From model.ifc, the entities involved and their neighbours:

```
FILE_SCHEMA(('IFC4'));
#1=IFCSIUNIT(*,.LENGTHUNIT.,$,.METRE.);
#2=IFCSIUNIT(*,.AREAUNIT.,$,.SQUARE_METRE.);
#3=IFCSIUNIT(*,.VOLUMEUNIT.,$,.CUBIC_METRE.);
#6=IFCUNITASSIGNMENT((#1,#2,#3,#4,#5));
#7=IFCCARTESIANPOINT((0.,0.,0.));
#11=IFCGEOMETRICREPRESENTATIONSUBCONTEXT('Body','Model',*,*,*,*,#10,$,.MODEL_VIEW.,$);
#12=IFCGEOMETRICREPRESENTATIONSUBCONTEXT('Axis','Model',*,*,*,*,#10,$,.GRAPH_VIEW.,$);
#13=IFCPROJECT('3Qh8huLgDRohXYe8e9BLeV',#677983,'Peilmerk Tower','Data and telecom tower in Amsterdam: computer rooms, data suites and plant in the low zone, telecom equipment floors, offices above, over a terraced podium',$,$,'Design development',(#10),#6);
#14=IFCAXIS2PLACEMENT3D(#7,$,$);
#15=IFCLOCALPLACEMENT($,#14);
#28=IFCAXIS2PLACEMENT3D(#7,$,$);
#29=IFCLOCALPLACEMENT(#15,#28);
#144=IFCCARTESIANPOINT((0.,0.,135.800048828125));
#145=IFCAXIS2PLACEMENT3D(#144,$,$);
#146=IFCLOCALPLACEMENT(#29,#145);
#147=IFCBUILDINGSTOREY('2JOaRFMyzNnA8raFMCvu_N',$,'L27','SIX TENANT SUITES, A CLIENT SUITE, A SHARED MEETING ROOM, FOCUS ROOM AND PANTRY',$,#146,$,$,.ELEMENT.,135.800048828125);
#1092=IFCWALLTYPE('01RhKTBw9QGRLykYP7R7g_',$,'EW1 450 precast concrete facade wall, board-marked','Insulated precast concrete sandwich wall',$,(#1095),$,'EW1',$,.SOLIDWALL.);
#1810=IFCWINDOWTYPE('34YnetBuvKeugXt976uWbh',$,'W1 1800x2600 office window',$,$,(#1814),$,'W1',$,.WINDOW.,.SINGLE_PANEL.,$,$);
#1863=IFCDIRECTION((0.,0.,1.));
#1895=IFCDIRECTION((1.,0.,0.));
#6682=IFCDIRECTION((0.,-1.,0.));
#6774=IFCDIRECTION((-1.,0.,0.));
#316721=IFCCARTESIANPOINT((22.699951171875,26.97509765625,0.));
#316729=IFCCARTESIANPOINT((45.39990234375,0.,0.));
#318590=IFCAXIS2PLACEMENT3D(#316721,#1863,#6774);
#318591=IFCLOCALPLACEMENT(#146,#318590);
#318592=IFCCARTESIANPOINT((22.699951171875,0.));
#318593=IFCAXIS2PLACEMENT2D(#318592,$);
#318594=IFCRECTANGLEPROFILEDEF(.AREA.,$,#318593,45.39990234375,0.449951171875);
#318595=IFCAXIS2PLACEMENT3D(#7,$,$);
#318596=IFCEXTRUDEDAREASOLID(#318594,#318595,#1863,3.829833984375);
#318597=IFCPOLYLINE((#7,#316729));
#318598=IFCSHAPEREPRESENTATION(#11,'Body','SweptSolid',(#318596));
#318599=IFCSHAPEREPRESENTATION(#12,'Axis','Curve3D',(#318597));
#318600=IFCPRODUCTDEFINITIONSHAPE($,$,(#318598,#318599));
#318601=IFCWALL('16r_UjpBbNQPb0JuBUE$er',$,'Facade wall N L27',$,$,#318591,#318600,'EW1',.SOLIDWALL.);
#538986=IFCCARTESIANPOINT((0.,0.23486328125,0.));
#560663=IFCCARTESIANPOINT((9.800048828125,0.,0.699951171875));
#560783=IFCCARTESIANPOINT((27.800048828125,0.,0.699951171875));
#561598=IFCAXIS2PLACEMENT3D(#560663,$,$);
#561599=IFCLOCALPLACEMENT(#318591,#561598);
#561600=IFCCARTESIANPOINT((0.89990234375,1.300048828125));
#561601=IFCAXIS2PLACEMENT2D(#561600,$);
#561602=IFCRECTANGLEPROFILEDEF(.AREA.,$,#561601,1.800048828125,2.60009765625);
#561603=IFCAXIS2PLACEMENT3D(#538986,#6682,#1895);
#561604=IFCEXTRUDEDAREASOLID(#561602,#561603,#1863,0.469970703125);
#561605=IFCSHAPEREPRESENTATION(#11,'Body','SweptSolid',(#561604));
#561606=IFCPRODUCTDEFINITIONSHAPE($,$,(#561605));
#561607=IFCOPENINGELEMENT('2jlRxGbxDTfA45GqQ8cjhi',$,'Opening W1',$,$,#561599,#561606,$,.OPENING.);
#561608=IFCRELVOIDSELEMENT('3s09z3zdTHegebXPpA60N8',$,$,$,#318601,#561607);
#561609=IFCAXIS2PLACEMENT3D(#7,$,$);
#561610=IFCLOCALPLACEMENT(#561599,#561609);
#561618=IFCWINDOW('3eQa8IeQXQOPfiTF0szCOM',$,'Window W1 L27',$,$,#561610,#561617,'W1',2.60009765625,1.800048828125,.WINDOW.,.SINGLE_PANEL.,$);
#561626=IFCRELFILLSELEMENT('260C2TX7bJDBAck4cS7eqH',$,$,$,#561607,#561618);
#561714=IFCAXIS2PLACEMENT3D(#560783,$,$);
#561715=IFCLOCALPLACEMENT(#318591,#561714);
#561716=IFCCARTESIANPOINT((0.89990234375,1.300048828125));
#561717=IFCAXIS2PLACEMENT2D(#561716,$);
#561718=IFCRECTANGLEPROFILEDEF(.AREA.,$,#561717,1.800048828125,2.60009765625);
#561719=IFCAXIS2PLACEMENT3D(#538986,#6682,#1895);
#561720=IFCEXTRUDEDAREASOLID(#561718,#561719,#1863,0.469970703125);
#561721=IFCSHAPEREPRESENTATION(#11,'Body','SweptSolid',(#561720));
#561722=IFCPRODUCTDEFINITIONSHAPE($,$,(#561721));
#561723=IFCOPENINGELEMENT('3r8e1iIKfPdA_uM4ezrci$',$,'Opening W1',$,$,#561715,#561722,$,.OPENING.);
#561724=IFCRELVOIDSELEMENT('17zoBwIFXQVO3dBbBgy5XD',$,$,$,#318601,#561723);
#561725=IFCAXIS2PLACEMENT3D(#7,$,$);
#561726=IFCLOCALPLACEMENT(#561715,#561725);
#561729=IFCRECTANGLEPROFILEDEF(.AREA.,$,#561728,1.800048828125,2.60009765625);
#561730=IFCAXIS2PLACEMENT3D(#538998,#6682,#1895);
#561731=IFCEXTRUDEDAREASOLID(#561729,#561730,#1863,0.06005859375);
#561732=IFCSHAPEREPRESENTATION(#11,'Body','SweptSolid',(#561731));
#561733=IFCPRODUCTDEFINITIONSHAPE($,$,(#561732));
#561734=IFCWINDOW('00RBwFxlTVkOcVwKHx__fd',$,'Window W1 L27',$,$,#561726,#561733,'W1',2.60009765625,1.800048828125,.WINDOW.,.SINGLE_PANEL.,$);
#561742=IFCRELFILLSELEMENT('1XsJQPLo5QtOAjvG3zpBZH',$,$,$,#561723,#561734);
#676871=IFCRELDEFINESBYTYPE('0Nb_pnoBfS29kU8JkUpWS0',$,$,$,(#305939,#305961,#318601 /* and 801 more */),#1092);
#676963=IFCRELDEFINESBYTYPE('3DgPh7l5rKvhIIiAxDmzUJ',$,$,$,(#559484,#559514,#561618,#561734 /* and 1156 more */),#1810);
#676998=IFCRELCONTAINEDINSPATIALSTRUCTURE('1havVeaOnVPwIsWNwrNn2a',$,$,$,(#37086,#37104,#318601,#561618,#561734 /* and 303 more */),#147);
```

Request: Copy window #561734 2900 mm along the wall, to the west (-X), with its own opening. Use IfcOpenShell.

```python
import ifcopenshell
import ifcopenshell.api.feature
import ifcopenshell.api.geometry
import ifcopenshell.api.root
import ifcopenshell.geom
import ifcopenshell.util.element
import ifcopenshell.util.placement
import ifcopenshell.util.shape
import ifcopenshell.util.unit

model = ifcopenshell.open("model.ifc")
unit_scale = ifcopenshell.util.unit.calculate_unit_scale(model)
settings = ifcopenshell.geom.settings()


def volume(element):
    """Net volume in cubic metres, openings subtracted."""
    shape = ifcopenshell.geom.create_shape(settings, element)
    return ifcopenshell.util.shape.get_volume(shape.geometry)


window = model.by_guid("00RBwFxlTVkOcVwKHx__fd")
opening = window.FillsVoids[0].RelatingOpeningElement
wall = opening.VoidsElements[0].RelatingBuildingElement
before = volume(wall)
shift = ifcopenshell.util.placement.get_local_placement(wall.ObjectPlacement)[:3, 0] * 2.9 / unit_scale

# copy_class copies the void relationship, type, container and properties, but no geometry.
new_opening = ifcopenshell.api.root.copy_class(model, product=opening)
new_opening.Representation = ifcopenshell.util.element.copy_deep(
    model, opening.Representation, exclude=["IfcGeometricRepresentationContext", "IfcRepresentationMap"]
)
new_window = ifcopenshell.api.root.copy_class(model, product=window)
new_window.Representation = ifcopenshell.util.element.copy_deep(
    model, window.Representation, exclude=["IfcGeometricRepresentationContext", "IfcRepresentationMap"]
)
new_window.Tag = None
ifcopenshell.api.feature.add_filling(model, opening=new_opening, element=new_window)

for old, new in ((opening, new_opening), (window, new_window)):
    matrix = ifcopenshell.util.placement.get_local_placement(old.ObjectPlacement)
    matrix[:3, 3] += shift
    ifcopenshell.api.geometry.edit_object_placement(model, product=new, matrix=matrix, is_si=False)

after = volume(wall)

print(f"wall volume {before:.3f} -> {after:.3f} m3")

model.write("model_rev.ifc")
```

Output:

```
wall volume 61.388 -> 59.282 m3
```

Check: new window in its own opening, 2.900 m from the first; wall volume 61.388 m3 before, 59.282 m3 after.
